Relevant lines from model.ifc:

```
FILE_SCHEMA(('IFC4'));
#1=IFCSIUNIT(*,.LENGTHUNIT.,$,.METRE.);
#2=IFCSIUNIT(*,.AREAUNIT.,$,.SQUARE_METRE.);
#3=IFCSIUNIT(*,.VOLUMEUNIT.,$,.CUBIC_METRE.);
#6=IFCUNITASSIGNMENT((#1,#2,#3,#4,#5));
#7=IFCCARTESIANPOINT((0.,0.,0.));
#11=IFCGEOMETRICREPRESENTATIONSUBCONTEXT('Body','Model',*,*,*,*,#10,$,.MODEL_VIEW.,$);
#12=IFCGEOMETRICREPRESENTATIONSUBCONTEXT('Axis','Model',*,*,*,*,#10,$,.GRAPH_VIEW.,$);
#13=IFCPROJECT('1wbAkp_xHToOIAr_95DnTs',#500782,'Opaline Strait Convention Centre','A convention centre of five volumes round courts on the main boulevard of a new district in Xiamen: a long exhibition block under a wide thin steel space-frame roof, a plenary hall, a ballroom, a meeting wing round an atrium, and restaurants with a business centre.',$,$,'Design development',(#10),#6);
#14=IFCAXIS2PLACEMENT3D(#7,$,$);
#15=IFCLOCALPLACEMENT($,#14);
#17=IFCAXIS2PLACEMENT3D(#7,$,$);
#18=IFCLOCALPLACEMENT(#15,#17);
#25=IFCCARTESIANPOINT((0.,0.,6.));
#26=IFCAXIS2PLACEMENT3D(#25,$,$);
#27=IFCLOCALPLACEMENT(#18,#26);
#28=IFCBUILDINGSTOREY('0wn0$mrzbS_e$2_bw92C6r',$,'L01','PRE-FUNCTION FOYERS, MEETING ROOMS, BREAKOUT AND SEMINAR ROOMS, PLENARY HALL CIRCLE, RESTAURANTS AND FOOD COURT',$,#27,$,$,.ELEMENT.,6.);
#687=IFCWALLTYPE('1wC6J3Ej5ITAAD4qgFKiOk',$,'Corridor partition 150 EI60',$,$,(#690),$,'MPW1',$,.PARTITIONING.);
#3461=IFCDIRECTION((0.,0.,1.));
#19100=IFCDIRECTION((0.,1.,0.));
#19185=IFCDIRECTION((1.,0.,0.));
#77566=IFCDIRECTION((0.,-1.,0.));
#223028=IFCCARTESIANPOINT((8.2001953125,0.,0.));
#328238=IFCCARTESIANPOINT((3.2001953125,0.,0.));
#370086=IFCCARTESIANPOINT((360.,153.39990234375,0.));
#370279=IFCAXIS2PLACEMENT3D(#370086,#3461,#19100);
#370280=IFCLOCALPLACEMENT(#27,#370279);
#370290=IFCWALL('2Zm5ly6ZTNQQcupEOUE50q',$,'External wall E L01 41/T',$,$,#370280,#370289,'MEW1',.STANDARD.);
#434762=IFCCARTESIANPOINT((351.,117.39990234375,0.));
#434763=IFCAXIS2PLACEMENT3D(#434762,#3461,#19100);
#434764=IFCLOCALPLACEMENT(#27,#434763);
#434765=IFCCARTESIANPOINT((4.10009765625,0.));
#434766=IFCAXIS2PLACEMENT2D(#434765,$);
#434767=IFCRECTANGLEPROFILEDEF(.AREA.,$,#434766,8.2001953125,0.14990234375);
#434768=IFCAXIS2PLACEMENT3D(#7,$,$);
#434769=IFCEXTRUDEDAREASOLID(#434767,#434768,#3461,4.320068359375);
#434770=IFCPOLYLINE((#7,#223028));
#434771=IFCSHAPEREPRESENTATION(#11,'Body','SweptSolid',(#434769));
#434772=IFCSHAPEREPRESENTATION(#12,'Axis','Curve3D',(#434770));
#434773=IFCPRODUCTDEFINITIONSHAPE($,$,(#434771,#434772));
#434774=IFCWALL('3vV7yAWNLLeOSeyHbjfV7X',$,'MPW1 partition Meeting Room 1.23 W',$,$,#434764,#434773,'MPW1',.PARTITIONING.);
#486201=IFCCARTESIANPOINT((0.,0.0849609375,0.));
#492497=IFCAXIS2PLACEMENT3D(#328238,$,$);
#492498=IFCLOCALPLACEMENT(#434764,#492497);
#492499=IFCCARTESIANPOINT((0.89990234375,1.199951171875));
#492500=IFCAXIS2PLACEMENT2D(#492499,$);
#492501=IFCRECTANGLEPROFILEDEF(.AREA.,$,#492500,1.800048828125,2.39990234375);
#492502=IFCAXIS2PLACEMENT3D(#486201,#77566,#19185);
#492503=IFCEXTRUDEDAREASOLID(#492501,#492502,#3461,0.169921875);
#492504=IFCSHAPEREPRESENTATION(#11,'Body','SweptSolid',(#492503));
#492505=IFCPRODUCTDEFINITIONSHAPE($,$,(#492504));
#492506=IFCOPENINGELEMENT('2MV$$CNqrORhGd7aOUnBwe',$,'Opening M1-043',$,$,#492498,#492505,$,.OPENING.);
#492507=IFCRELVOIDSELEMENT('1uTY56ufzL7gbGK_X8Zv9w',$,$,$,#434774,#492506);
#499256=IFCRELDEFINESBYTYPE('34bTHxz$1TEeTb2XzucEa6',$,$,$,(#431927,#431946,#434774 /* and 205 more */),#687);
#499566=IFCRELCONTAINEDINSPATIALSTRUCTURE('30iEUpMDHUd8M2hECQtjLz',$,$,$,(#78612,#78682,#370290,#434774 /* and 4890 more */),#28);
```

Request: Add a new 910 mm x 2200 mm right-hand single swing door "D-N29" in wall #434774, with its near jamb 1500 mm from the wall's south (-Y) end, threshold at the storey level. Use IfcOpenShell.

```python
import numpy as np
import ifcopenshell
import ifcopenshell.api.feature
import ifcopenshell.api.geometry
import ifcopenshell.api.root
import ifcopenshell.api.spatial
import ifcopenshell.geom
import ifcopenshell.util.element
import ifcopenshell.util.placement
import ifcopenshell.util.representation
import ifcopenshell.util.shape
import ifcopenshell.util.unit

model = ifcopenshell.open("model.ifc")
unit_scale = ifcopenshell.util.unit.calculate_unit_scale(model)
settings = ifcopenshell.geom.settings()


def volume(element):
    """Net volume in cubic metres, openings subtracted."""
    shape = ifcopenshell.geom.create_shape(settings, element)
    return ifcopenshell.util.shape.get_volume(shape.geometry)


wall = model.by_guid("3vV7yAWNLLeOSeyHbjfV7X")
storey = ifcopenshell.util.element.get_container(wall, ifc_class="IfcBuildingStorey")
context = ifcopenshell.util.representation.get_context(model, "Model", "Body", "MODEL_VIEW")
before = volume(wall)

width, height, from_end, sill = 0.91, 2.2, 1.5, 0.0  # metres

# The wall runs along its own X axis, and the end named is its -X end.
wall_shape = ifcopenshell.geom.create_shape(settings, wall)
x, y, z = ifcopenshell.util.shape.get_vertices(wall_shape.geometry).T
start = x.min() + from_end
face, thickness = float(y.min()), float(y.max() - y.min())
wall_matrix = ifcopenshell.util.placement.get_local_placement(wall.ObjectPlacement)
level = ifcopenshell.util.placement.get_local_placement(storey.ObjectPlacement)[2, 3]


def in_wall(x, y):
    """Placement at x, y metres in the wall's axes, at sill height."""
    matrix = wall_matrix.copy()
    matrix[:, 3] = wall_matrix @ np.array([x / unit_scale, y / unit_scale, 0.0, 1.0])
    matrix[2, 3] = level + sill / unit_scale
    return matrix


# Opening: a box that overshoots both wall faces by 50 mm.
opening = ifcopenshell.api.root.create_entity(model, ifc_class="IfcOpeningElement", predefined_type="OPENING")
box = ifcopenshell.api.geometry.add_wall_representation(
    model, context=context, length=width, height=height, thickness=thickness + 0.1
)
ifcopenshell.api.geometry.assign_representation(model, product=opening, representation=box)
ifcopenshell.api.geometry.edit_object_placement(model, product=opening, matrix=in_wall(start, face - 0.05), is_si=False)
ifcopenshell.api.feature.add_feature(model, feature=opening, element=wall)

door = ifcopenshell.api.root.create_entity(model, ifc_class="IfcDoor", name="D-N29", predefined_type="DOOR")
door.OverallWidth, door.OverallHeight = width / unit_scale, height / unit_scale
door.OperationType = "SINGLE_SWING_RIGHT"
body = ifcopenshell.api.geometry.add_door_representation(
    model,
    context=context,
    overall_width=door.OverallWidth,
    overall_height=door.OverallHeight,
    operation_type="SINGLE_SWING_RIGHT",
    lining_properties={"LiningDepth": thickness / unit_scale, "ThresholdDepth": thickness / unit_scale},
)
ifcopenshell.api.geometry.assign_representation(model, product=door, representation=body)
ifcopenshell.api.spatial.assign_container(model, products=[door], relating_structure=storey)
ifcopenshell.api.feature.add_filling(model, opening=opening, element=door)

# The lining spans the wall, so the door starts at the wall face.
ifcopenshell.api.geometry.edit_object_placement(model, product=door, matrix=in_wall(start, face), is_si=False)

after = volume(wall)

print(f"wall volume {before:.3f} -> {after:.3f} m3")

model.write("model_v2.ifc")
```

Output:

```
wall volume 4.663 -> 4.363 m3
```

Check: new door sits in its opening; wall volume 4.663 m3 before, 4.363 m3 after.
